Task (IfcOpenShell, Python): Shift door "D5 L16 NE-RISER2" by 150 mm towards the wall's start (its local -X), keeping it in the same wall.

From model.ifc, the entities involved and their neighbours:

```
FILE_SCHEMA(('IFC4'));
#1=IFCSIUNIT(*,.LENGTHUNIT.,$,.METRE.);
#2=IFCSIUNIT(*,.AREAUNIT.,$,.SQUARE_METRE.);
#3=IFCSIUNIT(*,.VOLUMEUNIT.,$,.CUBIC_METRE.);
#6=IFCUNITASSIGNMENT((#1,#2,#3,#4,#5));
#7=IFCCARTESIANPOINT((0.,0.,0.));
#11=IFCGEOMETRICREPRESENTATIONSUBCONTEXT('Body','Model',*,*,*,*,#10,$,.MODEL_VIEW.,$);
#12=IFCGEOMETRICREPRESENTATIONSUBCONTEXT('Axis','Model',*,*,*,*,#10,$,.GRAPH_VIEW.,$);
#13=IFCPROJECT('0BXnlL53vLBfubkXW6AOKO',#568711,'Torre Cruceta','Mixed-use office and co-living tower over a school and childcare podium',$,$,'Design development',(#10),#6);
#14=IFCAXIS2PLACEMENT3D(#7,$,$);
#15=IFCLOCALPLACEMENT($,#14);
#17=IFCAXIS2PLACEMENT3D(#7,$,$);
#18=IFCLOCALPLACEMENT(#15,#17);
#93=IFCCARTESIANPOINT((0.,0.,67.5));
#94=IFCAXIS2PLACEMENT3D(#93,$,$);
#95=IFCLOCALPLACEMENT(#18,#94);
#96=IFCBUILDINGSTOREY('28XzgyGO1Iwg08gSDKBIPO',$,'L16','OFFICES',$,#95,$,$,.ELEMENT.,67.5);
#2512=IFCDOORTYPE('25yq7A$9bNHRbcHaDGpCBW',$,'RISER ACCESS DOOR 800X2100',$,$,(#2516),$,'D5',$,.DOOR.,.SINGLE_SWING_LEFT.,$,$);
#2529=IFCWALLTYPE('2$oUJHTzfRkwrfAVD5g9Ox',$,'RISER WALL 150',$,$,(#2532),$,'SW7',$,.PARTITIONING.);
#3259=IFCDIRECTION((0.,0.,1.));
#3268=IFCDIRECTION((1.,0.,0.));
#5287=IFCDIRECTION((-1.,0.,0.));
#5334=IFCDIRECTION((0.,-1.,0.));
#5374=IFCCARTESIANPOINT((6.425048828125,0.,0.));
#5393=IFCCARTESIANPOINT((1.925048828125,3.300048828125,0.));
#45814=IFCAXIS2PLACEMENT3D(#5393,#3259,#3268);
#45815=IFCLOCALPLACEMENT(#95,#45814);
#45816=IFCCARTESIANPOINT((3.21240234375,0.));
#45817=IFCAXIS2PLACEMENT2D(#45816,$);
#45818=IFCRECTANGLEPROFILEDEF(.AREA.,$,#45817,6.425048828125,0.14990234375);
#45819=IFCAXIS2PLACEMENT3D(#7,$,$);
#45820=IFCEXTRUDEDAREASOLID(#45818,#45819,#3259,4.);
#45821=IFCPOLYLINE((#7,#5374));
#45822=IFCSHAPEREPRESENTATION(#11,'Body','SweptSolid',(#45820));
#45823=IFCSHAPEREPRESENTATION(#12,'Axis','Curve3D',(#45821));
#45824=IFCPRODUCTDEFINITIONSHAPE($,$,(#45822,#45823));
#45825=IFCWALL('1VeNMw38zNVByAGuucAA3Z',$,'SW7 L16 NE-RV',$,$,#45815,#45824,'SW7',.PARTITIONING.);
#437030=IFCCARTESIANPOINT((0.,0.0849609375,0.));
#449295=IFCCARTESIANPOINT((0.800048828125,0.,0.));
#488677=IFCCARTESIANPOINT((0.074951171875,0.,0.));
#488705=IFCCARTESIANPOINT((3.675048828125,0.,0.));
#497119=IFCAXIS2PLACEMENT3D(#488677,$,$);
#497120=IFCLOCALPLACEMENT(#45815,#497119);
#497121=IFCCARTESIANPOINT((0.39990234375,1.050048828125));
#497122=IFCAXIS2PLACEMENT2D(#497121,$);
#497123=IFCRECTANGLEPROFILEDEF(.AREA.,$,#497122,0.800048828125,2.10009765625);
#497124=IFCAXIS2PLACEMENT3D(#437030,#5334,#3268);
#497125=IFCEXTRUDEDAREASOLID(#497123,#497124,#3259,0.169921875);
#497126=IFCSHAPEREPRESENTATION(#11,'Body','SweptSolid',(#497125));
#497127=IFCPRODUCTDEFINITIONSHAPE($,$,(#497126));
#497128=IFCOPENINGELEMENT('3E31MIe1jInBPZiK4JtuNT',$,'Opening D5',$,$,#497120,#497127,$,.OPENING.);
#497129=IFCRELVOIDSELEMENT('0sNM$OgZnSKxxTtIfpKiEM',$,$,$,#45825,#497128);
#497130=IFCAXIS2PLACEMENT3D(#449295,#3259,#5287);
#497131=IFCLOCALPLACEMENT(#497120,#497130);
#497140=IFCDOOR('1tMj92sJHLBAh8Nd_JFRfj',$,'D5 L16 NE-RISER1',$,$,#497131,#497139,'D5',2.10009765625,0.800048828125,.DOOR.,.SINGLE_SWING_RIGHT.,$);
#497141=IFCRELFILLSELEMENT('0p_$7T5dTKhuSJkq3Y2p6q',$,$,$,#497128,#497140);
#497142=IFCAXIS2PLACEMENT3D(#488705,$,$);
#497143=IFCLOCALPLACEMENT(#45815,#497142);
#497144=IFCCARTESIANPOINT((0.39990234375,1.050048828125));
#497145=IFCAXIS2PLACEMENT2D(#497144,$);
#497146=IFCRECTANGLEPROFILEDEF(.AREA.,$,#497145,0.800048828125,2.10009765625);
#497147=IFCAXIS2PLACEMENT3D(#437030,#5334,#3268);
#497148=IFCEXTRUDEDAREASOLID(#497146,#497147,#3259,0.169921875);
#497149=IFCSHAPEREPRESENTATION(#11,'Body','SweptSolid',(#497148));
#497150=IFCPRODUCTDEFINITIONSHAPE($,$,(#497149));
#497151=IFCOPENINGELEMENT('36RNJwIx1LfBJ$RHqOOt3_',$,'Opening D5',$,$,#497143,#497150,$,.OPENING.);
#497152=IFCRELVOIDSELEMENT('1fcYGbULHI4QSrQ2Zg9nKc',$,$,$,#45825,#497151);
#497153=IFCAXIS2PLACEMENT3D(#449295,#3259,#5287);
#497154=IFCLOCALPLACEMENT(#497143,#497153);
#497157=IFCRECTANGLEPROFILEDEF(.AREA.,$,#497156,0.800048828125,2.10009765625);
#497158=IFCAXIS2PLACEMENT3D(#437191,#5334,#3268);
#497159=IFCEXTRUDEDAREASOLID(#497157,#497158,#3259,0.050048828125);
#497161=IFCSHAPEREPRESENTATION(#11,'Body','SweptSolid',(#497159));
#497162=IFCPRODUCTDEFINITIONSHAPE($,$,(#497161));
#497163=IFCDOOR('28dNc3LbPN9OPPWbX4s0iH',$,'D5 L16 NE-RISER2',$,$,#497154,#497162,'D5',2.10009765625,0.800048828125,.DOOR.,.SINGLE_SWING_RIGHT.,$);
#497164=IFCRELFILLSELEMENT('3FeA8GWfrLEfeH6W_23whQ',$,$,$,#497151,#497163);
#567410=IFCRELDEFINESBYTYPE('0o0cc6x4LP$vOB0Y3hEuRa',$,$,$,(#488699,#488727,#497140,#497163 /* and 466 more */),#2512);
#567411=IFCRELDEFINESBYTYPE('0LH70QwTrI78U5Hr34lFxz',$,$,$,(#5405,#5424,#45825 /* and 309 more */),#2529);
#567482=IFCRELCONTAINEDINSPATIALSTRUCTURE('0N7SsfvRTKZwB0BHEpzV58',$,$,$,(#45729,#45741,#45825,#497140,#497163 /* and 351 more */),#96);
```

```python
import ifcopenshell
import ifcopenshell.api.geometry
import ifcopenshell.util.placement
import ifcopenshell.util.unit

model = ifcopenshell.open("model.ifc")
unit_scale = ifcopenshell.util.unit.calculate_unit_scale(model)

door = model.by_guid("28dNc3LbPN9OPPWbX4s0iH")
opening = door.FillsVoids[0].RelatingOpeningElement
wall = opening.VoidsElements[0].RelatingBuildingElement

wall_matrix = ifcopenshell.util.placement.get_local_placement(wall.ObjectPlacement)
shift = wall_matrix[:3, 0] * -0.15 / unit_scale
before = ifcopenshell.util.placement.get_local_placement(door.ObjectPlacement)[:3, 3].copy()

# The door is placed relative to its opening, so it follows when the opening moves.
matrix = ifcopenshell.util.placement.get_local_placement(opening.ObjectPlacement)
matrix[:3, 3] += shift
ifcopenshell.api.geometry.edit_object_placement(
    model, product=opening, matrix=matrix, is_si=False, should_transform_children=True
)

after = ifcopenshell.util.placement.get_local_placement(door.ObjectPlacement)[:3, 3]
print("door moved by", (after - before).round(3) + 0.0)

model.write("model_v2.ifc")
```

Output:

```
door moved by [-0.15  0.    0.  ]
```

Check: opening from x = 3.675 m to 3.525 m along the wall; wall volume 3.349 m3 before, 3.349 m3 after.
